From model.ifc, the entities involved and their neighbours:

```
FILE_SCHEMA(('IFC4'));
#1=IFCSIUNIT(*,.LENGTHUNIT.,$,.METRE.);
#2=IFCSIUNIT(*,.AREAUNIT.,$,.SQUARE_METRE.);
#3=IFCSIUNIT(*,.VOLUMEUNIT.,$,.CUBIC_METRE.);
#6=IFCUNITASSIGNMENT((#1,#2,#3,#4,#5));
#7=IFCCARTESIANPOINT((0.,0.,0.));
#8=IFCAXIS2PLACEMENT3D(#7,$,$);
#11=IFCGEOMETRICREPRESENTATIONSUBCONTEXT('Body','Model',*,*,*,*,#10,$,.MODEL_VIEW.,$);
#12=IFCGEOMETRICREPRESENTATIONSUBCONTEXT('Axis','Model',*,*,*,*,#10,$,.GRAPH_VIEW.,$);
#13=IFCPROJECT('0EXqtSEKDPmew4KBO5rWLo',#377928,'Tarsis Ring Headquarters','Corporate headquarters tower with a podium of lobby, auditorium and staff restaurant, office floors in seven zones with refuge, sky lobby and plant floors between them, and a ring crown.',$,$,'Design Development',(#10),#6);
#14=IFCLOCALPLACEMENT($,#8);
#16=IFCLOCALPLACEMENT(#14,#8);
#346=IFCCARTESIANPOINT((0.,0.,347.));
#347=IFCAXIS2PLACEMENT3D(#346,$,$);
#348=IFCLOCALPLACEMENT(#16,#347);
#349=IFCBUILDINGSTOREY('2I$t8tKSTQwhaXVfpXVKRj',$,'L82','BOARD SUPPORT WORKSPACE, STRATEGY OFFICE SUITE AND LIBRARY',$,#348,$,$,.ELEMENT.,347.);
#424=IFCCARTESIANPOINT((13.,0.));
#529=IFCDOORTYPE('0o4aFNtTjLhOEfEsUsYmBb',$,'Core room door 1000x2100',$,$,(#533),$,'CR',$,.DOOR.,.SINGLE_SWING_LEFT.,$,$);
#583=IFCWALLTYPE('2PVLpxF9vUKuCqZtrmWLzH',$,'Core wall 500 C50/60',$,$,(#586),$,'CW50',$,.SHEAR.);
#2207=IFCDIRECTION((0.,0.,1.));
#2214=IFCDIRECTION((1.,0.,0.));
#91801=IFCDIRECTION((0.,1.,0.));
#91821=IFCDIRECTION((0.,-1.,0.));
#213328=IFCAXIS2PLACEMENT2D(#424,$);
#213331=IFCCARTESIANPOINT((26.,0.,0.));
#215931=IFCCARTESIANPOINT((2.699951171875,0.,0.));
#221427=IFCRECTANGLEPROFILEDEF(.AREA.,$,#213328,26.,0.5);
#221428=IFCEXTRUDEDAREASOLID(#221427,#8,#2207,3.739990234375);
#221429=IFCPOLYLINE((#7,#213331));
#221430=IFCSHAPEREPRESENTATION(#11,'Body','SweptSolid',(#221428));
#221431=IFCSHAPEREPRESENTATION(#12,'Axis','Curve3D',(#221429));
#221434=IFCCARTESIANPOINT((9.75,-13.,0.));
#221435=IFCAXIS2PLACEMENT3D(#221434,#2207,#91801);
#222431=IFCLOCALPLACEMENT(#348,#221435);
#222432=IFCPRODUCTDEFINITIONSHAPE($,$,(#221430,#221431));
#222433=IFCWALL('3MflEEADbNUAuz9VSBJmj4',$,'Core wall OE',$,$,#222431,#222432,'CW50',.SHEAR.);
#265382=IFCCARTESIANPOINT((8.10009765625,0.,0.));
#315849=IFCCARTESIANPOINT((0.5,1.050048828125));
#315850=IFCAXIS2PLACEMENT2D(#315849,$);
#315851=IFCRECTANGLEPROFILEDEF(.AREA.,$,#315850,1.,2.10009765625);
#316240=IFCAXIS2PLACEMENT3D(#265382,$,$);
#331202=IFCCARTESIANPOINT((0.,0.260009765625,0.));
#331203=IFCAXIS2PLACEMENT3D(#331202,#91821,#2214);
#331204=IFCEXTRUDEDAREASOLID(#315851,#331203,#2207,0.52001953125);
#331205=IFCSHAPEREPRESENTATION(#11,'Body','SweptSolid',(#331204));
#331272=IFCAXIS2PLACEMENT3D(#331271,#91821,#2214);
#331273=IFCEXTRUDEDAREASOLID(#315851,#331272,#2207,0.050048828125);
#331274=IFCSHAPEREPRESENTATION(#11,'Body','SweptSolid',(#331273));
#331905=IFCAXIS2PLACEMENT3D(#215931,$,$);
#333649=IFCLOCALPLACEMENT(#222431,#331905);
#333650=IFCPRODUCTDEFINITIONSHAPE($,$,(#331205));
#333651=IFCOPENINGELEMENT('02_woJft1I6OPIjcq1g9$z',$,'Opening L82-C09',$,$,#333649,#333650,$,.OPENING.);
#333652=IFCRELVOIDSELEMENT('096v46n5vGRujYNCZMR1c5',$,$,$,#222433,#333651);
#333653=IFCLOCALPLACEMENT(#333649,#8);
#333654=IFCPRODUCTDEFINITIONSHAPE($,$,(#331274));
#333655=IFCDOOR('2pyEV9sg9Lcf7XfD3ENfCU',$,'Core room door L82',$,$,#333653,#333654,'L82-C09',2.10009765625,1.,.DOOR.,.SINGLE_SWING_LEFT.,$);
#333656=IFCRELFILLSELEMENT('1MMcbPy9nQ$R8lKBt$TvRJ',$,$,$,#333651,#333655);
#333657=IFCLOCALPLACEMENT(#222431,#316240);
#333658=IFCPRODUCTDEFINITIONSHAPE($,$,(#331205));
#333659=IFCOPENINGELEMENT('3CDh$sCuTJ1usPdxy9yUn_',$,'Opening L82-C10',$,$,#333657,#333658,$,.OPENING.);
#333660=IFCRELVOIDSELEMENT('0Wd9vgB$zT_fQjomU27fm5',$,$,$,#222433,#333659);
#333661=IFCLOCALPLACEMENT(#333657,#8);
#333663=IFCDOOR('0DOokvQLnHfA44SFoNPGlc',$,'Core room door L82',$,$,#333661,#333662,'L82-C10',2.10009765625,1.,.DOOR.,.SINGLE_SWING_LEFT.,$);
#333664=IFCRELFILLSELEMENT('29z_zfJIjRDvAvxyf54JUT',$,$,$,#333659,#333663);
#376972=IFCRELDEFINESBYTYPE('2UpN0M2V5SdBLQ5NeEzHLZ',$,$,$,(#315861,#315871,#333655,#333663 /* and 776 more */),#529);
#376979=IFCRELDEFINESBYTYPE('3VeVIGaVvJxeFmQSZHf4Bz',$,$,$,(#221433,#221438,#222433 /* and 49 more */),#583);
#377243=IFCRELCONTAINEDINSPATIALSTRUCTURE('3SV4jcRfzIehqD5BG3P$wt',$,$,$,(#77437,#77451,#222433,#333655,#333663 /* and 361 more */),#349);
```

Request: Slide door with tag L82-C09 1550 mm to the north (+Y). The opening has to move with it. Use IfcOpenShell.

```python
import ifcopenshell
import ifcopenshell.api.geometry
import ifcopenshell.util.placement

model = ifcopenshell.open("model.ifc")

door = model.by_guid("2pyEV9sg9Lcf7XfD3ENfCU")
opening = door.FillsVoids[0].RelatingOpeningElement
wall = opening.VoidsElements[0].RelatingBuildingElement

wall_matrix = ifcopenshell.util.placement.get_local_placement(wall.ObjectPlacement)
shift = wall_matrix[:3, 0] * 1.55
before = ifcopenshell.util.placement.get_local_placement(door.ObjectPlacement)[:3, 3].copy()

# The door is placed relative to its opening, so it follows when the opening moves.
matrix = ifcopenshell.util.placement.get_local_placement(opening.ObjectPlacement)
matrix[:3, 3] += shift
ifcopenshell.api.geometry.edit_object_placement(
    model, product=opening, matrix=matrix, is_si=False, should_transform_children=True
)

after = ifcopenshell.util.placement.get_local_placement(door.ObjectPlacement)[:3, 3]
print("door moved by", (after - before).round(3) + 0.0)

model.write("model_edited.ifc")
```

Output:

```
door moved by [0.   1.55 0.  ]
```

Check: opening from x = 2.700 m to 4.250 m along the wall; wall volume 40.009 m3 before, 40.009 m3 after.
